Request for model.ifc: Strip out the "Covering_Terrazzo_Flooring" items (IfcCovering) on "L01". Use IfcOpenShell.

First a look at what the model holds.

```python
import ifcopenshell
import ifcopenshell.util.element

model = ifcopenshell.open("model.ifc")
print(model.schema)
storey = next(s for s in model.by_type("IfcBuildingStorey") if s.Name == "L01")
coverings = [e for e in ifcopenshell.util.element.get_decomposition(storey) if e.is_a("IfcCovering")]
seen = {}
for e in coverings:
    element_type = ifcopenshell.util.element.get_type(e)
    name = element_type.Name if element_type not in (None, e) else None
    seen[name] = seen.get(name, 0) + 1
for name, count in sorted(seen.items(), key=str):
    print(count, "x", name)
```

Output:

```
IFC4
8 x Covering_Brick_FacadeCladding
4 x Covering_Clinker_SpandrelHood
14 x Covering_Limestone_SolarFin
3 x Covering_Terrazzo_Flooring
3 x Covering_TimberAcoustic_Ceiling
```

```python
import ifcopenshell
import ifcopenshell.api.root
import ifcopenshell.util.element

model = ifcopenshell.open("model.ifc")

storey = next(s for s in model.by_type("IfcBuildingStorey") if s.Name == "L01")
coverings = [e for e in ifcopenshell.util.element.get_decomposition(storey) if e.is_a("IfcCovering")]
targets = [e for e in coverings if (t := ifcopenshell.util.element.get_type(e)) not in (None, e) and t.Name == "Covering_Terrazzo_Flooring"]

for e in targets:
    ifcopenshell.api.root.remove_product(model, product=e)
print(len(targets), "removed")

model.write("model-out.ifc")
```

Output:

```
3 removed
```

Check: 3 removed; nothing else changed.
